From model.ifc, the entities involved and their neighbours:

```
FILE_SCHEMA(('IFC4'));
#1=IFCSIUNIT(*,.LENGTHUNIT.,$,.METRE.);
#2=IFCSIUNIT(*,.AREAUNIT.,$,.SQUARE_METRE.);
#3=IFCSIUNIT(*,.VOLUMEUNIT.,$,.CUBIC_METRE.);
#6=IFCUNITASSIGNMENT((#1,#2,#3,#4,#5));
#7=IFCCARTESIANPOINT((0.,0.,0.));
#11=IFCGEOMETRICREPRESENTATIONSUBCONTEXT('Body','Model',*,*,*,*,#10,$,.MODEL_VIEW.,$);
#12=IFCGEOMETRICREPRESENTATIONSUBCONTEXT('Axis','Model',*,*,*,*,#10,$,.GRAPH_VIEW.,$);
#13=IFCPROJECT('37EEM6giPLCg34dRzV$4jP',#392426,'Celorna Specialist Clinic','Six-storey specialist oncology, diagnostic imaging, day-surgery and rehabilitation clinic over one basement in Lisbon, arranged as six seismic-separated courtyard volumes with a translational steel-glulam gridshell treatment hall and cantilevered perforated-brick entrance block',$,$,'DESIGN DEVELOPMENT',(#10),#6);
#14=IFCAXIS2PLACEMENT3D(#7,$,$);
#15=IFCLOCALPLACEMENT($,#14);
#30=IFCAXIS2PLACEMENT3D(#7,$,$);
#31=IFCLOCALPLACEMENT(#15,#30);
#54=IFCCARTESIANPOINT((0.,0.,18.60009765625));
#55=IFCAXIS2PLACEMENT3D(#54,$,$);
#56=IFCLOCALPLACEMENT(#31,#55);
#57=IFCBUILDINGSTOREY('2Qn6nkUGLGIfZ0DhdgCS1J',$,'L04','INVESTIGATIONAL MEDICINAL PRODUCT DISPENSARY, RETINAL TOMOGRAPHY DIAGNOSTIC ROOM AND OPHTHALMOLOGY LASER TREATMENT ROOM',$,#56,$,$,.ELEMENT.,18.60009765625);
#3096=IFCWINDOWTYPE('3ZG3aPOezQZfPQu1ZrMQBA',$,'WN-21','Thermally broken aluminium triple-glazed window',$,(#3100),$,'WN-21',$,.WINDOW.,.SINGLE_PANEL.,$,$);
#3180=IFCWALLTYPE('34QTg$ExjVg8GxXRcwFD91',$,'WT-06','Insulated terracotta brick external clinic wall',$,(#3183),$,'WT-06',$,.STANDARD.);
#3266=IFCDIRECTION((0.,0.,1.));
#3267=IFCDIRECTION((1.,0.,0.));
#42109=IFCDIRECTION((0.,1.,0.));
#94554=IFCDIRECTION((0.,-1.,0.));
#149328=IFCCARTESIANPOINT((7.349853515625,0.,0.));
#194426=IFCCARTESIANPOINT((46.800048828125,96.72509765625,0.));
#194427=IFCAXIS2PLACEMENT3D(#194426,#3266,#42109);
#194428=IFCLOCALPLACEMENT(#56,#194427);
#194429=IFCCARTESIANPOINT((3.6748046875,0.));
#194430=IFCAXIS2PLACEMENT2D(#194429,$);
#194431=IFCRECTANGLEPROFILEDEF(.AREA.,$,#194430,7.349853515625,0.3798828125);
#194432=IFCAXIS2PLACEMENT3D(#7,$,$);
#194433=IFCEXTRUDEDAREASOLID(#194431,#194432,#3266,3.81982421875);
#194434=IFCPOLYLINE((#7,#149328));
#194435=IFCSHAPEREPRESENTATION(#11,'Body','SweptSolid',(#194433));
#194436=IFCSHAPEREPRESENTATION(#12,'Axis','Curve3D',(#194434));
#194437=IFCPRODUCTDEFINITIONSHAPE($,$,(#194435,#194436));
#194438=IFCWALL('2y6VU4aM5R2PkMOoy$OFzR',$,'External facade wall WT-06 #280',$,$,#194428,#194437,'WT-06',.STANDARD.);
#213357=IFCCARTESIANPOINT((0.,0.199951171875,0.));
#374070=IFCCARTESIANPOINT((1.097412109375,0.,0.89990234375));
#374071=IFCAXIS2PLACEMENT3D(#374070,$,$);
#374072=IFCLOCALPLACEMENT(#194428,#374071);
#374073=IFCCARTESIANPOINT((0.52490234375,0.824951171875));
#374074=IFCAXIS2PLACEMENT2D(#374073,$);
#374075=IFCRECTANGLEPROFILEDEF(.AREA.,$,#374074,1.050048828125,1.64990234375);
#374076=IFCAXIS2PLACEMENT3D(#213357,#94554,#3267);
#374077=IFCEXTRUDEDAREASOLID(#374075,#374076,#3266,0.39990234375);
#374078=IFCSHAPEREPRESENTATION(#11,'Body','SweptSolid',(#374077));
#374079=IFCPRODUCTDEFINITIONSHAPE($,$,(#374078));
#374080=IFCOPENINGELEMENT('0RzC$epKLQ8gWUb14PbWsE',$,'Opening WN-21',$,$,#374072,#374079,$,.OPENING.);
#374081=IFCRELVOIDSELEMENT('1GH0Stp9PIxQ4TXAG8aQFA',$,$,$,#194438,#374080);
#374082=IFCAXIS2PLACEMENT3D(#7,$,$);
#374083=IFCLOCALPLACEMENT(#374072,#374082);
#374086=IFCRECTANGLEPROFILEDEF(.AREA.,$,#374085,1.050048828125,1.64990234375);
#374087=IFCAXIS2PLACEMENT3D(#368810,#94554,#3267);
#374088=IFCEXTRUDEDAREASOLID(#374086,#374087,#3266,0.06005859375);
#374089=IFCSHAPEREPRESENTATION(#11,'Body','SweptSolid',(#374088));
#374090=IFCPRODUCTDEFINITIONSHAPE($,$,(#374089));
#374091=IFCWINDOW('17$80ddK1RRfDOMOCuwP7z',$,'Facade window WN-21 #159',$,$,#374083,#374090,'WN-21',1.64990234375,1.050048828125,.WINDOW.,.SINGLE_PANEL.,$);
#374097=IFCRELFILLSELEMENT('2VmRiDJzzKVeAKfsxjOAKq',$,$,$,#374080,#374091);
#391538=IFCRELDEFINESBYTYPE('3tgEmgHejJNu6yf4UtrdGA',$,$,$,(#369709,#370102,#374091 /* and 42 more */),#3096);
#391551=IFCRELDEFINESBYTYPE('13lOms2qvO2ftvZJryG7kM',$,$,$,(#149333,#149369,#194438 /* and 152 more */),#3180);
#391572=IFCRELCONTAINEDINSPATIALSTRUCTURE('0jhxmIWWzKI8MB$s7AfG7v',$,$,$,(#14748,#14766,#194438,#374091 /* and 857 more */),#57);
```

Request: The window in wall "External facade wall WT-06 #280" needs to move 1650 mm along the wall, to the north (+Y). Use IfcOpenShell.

```python
import ifcopenshell
import ifcopenshell.api.geometry
import ifcopenshell.util.placement

model = ifcopenshell.open("model.ifc")

window = model.by_guid("17$80ddK1RRfDOMOCuwP7z")
opening = window.FillsVoids[0].RelatingOpeningElement
wall = opening.VoidsElements[0].RelatingBuildingElement

wall_matrix = ifcopenshell.util.placement.get_local_placement(wall.ObjectPlacement)
shift = wall_matrix[:3, 0] * 1.65
before = ifcopenshell.util.placement.get_local_placement(window.ObjectPlacement)[:3, 3].copy()

# The window is placed relative to its opening, so it follows when the opening moves.
matrix = ifcopenshell.util.placement.get_local_placement(opening.ObjectPlacement)
matrix[:3, 3] += shift
ifcopenshell.api.geometry.edit_object_placement(
    model, product=opening, matrix=matrix, is_si=False, should_transform_children=True
)

after = ifcopenshell.util.placement.get_local_placement(window.ObjectPlacement)[:3, 3]
print("window moved by", (after - before).round(3) + 0.0)

model.write("model_updated.ifc")
```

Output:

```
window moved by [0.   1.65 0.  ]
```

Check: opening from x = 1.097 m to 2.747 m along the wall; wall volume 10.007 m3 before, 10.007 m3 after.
